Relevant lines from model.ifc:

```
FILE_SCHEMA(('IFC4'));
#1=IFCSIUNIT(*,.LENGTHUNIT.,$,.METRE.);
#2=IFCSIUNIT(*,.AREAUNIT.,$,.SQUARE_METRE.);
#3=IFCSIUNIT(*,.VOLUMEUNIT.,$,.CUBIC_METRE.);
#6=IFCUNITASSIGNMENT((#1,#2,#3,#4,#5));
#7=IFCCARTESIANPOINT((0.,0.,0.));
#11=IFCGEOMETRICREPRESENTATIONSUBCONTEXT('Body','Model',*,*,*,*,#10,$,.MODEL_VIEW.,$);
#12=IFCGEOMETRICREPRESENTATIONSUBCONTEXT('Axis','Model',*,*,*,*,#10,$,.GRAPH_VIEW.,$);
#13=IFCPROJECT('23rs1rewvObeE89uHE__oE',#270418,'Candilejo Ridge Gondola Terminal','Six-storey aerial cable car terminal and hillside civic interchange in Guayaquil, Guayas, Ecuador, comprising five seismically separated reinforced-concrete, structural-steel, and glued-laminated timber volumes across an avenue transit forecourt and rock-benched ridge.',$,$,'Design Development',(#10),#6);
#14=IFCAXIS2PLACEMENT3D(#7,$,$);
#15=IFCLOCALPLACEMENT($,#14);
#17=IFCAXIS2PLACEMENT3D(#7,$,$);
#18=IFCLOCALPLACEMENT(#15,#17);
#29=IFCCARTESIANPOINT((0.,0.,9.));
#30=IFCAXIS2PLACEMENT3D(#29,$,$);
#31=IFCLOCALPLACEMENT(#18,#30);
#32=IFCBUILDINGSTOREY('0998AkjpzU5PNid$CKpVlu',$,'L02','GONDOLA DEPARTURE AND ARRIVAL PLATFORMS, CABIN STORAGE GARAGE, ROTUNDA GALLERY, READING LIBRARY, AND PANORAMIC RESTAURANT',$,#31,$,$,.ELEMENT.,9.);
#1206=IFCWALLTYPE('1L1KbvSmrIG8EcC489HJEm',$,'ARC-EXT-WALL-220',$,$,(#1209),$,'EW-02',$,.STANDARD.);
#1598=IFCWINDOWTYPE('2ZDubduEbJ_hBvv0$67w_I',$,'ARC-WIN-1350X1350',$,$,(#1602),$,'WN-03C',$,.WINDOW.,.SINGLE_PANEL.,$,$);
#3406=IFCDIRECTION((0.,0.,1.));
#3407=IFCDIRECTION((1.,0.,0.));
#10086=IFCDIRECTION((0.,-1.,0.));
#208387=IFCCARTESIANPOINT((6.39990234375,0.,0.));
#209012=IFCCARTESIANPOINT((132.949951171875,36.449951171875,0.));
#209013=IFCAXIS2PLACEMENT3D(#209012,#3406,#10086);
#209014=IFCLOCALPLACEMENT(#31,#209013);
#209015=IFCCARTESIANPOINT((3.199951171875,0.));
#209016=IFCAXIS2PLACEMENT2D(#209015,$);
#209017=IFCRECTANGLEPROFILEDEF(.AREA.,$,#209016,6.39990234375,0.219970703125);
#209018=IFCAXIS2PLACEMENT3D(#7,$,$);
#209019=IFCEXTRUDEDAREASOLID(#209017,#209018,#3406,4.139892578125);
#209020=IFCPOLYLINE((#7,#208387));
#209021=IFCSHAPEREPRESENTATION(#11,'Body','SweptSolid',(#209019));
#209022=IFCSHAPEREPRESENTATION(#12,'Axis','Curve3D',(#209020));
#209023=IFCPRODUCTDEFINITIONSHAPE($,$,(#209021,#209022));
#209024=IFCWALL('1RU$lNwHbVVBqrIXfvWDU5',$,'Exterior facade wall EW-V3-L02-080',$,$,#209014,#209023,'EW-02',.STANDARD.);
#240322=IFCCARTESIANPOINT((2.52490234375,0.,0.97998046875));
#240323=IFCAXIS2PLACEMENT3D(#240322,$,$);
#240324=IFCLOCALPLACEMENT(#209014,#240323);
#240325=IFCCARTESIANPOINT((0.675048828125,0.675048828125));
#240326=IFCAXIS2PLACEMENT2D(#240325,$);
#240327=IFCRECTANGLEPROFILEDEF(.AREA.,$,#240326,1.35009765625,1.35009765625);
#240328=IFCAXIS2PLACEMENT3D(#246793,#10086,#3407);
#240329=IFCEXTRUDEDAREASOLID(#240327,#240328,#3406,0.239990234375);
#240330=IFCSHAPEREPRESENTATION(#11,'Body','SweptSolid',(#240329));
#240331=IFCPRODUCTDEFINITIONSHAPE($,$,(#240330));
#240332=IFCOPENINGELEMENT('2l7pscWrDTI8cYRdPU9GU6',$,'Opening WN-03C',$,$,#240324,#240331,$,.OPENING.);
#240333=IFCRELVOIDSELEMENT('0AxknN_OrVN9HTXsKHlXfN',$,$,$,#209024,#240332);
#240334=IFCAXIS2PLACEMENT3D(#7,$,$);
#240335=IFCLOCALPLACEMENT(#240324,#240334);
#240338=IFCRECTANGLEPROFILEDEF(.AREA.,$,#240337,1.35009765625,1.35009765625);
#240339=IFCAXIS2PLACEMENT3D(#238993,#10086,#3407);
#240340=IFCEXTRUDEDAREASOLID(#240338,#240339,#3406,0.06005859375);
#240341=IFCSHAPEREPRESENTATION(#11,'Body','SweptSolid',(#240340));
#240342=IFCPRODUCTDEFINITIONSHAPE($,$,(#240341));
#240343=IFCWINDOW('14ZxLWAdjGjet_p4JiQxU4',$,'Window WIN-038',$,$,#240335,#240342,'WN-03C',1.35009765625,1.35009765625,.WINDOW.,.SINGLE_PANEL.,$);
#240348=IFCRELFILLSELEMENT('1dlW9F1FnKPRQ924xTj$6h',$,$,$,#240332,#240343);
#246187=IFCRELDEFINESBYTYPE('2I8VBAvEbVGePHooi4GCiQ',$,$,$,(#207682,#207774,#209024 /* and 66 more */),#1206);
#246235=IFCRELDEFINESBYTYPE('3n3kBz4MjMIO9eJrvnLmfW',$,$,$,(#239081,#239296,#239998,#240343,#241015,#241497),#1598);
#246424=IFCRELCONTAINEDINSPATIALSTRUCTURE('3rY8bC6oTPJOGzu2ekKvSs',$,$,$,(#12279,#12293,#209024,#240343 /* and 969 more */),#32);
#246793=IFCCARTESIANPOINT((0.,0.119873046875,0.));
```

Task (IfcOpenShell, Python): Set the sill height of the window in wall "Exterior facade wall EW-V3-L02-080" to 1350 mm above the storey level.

```python
import numpy as np
import ifcopenshell
import ifcopenshell.api.geometry
import ifcopenshell.geom
import ifcopenshell.util.element
import ifcopenshell.util.placement
import ifcopenshell.util.shape
import ifcopenshell.util.unit

model = ifcopenshell.open("model.ifc")
unit_scale = ifcopenshell.util.unit.calculate_unit_scale(model)

window = model.by_id(240343)
opening = window.FillsVoids[0].RelatingOpeningElement
storey = ifcopenshell.util.element.get_container(window, ifc_class="IfcBuildingStorey")
level = ifcopenshell.util.placement.get_local_placement(storey.ObjectPlacement)[2, 3]

# The opening's origin need not be at the sill, so measure its lowest point.
shape = ifcopenshell.geom.create_shape(ifcopenshell.geom.settings(), opening)
bottom = ifcopenshell.util.shape.get_shape_bottom_elevation(shape, shape.geometry) / unit_scale
dz = level + 1.35 / unit_scale - bottom

shift = np.array([0.0, 0.0, dz])
# The window is placed relative to its opening, so it follows when the opening moves.
matrix = ifcopenshell.util.placement.get_local_placement(opening.ObjectPlacement)
matrix[:3, 3] += shift
ifcopenshell.api.geometry.edit_object_placement(
    model, product=opening, matrix=matrix, is_si=False, should_transform_children=True
)

print(f"moved by {dz * unit_scale:+.3f} m")

model.write("model-out.ifc")
```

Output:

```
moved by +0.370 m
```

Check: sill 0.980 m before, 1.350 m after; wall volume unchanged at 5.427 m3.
